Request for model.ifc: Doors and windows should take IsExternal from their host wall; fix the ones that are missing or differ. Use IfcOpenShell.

First a look at what the model holds.

```python
import ifcopenshell
import ifcopenshell.util.element

model = ifcopenshell.open("model.ifc")
print(model.schema)
seen = {}
for e in model.by_type("IfcDoor") + model.by_type("IfcWindow"):
    if not e.FillsVoids:
        continue
    host = e.FillsVoids[0].RelatingOpeningElement.VoidsElements[0].RelatingBuildingElement
    own = ifcopenshell.util.element.get_pset(e, f"Pset_{e.is_a()[3:].removesuffix('StandardCase')}Common", "IsExternal")
    wall = ifcopenshell.util.element.get_pset(host, "Pset_WallCommon", "IsExternal")
    seen[e.is_a(), own, wall] = seen.get((e.is_a(), own, wall), 0) + 1
for (cls, own, wall), count in sorted(seen.items(), key=str):
    print(count, cls, "IsExternal:", own, "| host wall:", wall)
```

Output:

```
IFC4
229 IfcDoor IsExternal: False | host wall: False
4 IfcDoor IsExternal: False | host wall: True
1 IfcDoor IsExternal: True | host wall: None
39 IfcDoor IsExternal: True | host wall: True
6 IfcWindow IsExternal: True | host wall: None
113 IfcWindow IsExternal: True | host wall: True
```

```python
import ifcopenshell
import ifcopenshell.api.pset
import ifcopenshell.util.element

model = ifcopenshell.open("model.ifc")

count = 0
for ifc_class, pset_name in (("IfcDoor", "Pset_DoorCommon"), ("IfcWindow", "Pset_WindowCommon")):
    for e in model.by_type(ifc_class):
        if not e.FillsVoids:
            continue
        host = e.FillsVoids[0].RelatingOpeningElement.VoidsElements[0].RelatingBuildingElement
        external = ifcopenshell.util.element.get_pset(host, "Pset_WallCommon", "IsExternal")
        if external is None or ifcopenshell.util.element.get_pset(e, pset_name, "IsExternal") == external:
            continue
        pset = ifcopenshell.api.pset.add_pset(model, product=e, name=pset_name)
        ifcopenshell.api.pset.edit_pset(model, pset=pset, properties={"IsExternal": external})
        count += 1

print(count, "updated")

model.write("model_edited.ifc")
```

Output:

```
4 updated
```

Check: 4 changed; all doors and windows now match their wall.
